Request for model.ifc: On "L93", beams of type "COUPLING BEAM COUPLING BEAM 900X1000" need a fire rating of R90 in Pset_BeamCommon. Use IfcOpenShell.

First a look at what the model holds.

```python
import ifcopenshell
import ifcopenshell.util.element

model = ifcopenshell.open("model.ifc")
print(model.schema)
storey = next(s for s in model.by_type("IfcBuildingStorey") if s.Name == "L93")
beams = [e for e in ifcopenshell.util.element.get_decomposition(storey) if e.is_a("IfcBeam")]
seen = {}
for e in beams:
    element_type = ifcopenshell.util.element.get_type(e)
    key = (element_type.Name if element_type != e and element_type else None, ifcopenshell.util.element.get_pset(e, "Pset_BeamCommon", "FireRating"))
    seen[key] = seen.get(key, 0) + 1
for (name, value), count in sorted(seen.items(), key=str):
    print(count, "x", name, "|", value)
```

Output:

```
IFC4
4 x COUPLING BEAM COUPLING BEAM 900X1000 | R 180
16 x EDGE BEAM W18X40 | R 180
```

```python
import ifcopenshell
import ifcopenshell.api.pset
import ifcopenshell.util.element

model = ifcopenshell.open("model.ifc")

storey = next(s for s in model.by_type("IfcBuildingStorey") if s.Name == "L93")
beams = [e for e in ifcopenshell.util.element.get_decomposition(storey) if e.is_a("IfcBeam")]

count = 0
for e in beams:
    element_type = ifcopenshell.util.element.get_type(e)
    if element_type in (None, e) or element_type.Name != "COUPLING BEAM COUPLING BEAM 900X1000":
        continue
    found = ifcopenshell.util.element.get_pset(e, "Pset_BeamCommon", should_inherit=False)
    if found:
        pset = model.by_id(found["id"])
        if len(ifcopenshell.util.element.get_elements_by_pset(pset)) > 1:
            pset = ifcopenshell.api.pset.unshare_pset(model, products=[e], pset=pset)[0]
    else:
        pset = ifcopenshell.api.pset.add_pset(model, product=e, name="Pset_BeamCommon")
    ifcopenshell.api.pset.edit_pset(model, pset=pset, properties={"FireRating": "R90"})
    count += 1

print(count, "beams updated")

model.write("model_v2.ifc")
```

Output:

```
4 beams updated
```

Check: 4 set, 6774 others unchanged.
